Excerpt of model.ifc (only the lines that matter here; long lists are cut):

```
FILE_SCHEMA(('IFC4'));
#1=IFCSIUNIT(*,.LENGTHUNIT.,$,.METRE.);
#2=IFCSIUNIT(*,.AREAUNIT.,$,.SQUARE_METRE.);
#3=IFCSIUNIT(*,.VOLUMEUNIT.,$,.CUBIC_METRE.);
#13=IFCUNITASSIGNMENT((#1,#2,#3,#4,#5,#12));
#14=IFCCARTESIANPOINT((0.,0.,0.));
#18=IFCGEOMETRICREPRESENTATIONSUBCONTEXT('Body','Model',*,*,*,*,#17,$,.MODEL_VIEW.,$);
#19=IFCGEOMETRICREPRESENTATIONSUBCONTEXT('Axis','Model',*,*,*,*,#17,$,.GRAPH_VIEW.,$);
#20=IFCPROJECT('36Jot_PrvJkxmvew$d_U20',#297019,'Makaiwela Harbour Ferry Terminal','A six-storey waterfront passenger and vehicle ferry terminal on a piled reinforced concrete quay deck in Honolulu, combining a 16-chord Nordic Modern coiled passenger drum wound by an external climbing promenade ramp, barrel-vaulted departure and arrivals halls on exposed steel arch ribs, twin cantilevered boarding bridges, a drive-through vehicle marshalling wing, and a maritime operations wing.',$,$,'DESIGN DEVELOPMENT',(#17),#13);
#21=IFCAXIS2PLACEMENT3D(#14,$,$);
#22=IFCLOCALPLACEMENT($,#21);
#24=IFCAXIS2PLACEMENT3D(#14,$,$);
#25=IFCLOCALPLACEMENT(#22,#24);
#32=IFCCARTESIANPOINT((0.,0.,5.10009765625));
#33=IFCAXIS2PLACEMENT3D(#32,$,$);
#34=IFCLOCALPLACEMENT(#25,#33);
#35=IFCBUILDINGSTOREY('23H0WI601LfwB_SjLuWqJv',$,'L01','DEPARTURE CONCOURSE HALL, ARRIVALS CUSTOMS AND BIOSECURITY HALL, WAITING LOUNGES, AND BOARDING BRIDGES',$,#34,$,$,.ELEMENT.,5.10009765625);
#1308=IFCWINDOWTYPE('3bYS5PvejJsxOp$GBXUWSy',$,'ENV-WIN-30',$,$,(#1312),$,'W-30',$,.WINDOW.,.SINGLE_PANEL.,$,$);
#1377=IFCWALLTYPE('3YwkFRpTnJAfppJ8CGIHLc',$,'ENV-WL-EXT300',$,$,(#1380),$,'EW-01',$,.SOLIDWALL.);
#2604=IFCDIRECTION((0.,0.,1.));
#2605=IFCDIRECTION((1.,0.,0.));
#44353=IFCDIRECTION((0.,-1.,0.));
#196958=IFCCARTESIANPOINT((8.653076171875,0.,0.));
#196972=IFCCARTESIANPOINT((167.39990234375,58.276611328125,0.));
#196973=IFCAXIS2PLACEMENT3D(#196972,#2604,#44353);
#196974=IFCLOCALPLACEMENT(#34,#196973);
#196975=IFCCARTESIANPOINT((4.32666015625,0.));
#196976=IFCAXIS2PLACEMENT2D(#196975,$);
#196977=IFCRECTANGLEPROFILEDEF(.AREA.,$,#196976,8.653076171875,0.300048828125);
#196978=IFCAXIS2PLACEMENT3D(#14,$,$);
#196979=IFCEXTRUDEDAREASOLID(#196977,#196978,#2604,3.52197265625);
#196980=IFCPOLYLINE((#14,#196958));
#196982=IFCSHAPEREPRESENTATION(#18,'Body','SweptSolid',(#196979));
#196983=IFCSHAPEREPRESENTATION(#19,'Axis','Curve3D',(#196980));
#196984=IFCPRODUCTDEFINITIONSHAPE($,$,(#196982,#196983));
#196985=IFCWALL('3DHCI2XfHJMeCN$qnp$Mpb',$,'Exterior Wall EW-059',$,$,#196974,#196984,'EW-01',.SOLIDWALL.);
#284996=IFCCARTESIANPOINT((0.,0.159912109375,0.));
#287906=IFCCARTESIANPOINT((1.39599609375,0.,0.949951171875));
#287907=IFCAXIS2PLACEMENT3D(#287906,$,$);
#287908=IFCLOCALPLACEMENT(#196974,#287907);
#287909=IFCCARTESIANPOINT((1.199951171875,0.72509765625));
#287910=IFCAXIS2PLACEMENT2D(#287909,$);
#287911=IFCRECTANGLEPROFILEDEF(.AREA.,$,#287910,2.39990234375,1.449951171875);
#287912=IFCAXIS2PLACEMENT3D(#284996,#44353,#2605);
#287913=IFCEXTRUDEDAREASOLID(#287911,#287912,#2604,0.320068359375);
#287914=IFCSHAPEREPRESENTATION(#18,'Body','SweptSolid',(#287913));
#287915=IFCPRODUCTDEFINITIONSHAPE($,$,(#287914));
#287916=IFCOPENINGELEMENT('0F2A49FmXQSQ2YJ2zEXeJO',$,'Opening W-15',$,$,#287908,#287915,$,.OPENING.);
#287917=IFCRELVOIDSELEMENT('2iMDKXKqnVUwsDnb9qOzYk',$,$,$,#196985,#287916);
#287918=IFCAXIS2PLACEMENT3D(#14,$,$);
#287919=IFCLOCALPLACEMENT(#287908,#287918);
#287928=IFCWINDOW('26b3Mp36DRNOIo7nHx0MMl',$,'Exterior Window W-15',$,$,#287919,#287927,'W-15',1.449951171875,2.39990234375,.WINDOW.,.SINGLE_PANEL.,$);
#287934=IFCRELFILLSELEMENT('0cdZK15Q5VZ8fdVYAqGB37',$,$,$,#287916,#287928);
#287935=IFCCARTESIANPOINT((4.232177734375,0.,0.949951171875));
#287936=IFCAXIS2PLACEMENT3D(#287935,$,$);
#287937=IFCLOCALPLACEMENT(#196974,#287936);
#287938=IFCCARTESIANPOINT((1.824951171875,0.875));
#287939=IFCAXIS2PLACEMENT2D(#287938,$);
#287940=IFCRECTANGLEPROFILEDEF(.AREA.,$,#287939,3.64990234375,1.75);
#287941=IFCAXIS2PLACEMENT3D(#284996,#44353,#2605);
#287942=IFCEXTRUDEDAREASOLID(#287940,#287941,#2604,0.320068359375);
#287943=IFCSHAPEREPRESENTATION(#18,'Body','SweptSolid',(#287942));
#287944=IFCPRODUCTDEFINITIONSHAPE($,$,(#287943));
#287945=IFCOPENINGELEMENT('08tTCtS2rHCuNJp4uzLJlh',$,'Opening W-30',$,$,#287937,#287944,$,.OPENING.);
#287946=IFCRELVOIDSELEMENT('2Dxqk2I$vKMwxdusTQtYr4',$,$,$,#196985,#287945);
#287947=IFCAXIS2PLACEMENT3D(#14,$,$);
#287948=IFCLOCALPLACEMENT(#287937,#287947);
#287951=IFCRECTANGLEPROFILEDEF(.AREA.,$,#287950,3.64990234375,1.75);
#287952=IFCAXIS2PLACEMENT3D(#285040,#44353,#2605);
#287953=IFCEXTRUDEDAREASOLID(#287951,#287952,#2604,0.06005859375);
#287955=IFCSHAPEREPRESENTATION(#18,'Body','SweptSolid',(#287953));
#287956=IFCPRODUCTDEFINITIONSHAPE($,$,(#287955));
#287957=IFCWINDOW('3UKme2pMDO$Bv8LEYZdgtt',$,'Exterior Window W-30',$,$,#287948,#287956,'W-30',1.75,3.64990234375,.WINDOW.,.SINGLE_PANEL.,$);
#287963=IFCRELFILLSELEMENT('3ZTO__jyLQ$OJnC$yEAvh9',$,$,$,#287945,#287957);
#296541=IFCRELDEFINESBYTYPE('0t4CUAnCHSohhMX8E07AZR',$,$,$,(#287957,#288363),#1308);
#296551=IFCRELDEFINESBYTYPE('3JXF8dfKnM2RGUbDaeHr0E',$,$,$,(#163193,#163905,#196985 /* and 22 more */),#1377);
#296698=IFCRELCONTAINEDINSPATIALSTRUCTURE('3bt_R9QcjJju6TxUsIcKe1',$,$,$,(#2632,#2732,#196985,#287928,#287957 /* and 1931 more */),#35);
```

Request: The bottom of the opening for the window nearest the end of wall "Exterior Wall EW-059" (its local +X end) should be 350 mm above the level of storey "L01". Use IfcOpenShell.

```python
import numpy as np
import ifcopenshell
import ifcopenshell.api.geometry
import ifcopenshell.geom
import ifcopenshell.util.element
import ifcopenshell.util.placement
import ifcopenshell.util.shape
import ifcopenshell.util.unit

model = ifcopenshell.open("model.ifc")
unit_scale = ifcopenshell.util.unit.calculate_unit_scale(model)

window = model.by_guid("3UKme2pMDO$Bv8LEYZdgtt")
opening = window.FillsVoids[0].RelatingOpeningElement
storey = ifcopenshell.util.element.get_container(window, ifc_class="IfcBuildingStorey")
level = ifcopenshell.util.placement.get_local_placement(storey.ObjectPlacement)[2, 3]

# The opening's origin need not be at the sill, so measure its lowest point.
shape = ifcopenshell.geom.create_shape(ifcopenshell.geom.settings(), opening)
bottom = ifcopenshell.util.shape.get_shape_bottom_elevation(shape, shape.geometry) / unit_scale
dz = level + 0.35 / unit_scale - bottom

shift = np.array([0.0, 0.0, dz])
# The window is placed relative to its opening, so it follows when the opening moves.
matrix = ifcopenshell.util.placement.get_local_placement(opening.ObjectPlacement)
matrix[:3, 3] += shift
ifcopenshell.api.geometry.edit_object_placement(
    model, product=opening, matrix=matrix, is_si=False, should_transform_children=True
)

print(f"moved by {dz * unit_scale:+.3f} m")

model.write("model_updated.ifc")
```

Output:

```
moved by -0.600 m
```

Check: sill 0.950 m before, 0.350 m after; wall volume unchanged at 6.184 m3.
